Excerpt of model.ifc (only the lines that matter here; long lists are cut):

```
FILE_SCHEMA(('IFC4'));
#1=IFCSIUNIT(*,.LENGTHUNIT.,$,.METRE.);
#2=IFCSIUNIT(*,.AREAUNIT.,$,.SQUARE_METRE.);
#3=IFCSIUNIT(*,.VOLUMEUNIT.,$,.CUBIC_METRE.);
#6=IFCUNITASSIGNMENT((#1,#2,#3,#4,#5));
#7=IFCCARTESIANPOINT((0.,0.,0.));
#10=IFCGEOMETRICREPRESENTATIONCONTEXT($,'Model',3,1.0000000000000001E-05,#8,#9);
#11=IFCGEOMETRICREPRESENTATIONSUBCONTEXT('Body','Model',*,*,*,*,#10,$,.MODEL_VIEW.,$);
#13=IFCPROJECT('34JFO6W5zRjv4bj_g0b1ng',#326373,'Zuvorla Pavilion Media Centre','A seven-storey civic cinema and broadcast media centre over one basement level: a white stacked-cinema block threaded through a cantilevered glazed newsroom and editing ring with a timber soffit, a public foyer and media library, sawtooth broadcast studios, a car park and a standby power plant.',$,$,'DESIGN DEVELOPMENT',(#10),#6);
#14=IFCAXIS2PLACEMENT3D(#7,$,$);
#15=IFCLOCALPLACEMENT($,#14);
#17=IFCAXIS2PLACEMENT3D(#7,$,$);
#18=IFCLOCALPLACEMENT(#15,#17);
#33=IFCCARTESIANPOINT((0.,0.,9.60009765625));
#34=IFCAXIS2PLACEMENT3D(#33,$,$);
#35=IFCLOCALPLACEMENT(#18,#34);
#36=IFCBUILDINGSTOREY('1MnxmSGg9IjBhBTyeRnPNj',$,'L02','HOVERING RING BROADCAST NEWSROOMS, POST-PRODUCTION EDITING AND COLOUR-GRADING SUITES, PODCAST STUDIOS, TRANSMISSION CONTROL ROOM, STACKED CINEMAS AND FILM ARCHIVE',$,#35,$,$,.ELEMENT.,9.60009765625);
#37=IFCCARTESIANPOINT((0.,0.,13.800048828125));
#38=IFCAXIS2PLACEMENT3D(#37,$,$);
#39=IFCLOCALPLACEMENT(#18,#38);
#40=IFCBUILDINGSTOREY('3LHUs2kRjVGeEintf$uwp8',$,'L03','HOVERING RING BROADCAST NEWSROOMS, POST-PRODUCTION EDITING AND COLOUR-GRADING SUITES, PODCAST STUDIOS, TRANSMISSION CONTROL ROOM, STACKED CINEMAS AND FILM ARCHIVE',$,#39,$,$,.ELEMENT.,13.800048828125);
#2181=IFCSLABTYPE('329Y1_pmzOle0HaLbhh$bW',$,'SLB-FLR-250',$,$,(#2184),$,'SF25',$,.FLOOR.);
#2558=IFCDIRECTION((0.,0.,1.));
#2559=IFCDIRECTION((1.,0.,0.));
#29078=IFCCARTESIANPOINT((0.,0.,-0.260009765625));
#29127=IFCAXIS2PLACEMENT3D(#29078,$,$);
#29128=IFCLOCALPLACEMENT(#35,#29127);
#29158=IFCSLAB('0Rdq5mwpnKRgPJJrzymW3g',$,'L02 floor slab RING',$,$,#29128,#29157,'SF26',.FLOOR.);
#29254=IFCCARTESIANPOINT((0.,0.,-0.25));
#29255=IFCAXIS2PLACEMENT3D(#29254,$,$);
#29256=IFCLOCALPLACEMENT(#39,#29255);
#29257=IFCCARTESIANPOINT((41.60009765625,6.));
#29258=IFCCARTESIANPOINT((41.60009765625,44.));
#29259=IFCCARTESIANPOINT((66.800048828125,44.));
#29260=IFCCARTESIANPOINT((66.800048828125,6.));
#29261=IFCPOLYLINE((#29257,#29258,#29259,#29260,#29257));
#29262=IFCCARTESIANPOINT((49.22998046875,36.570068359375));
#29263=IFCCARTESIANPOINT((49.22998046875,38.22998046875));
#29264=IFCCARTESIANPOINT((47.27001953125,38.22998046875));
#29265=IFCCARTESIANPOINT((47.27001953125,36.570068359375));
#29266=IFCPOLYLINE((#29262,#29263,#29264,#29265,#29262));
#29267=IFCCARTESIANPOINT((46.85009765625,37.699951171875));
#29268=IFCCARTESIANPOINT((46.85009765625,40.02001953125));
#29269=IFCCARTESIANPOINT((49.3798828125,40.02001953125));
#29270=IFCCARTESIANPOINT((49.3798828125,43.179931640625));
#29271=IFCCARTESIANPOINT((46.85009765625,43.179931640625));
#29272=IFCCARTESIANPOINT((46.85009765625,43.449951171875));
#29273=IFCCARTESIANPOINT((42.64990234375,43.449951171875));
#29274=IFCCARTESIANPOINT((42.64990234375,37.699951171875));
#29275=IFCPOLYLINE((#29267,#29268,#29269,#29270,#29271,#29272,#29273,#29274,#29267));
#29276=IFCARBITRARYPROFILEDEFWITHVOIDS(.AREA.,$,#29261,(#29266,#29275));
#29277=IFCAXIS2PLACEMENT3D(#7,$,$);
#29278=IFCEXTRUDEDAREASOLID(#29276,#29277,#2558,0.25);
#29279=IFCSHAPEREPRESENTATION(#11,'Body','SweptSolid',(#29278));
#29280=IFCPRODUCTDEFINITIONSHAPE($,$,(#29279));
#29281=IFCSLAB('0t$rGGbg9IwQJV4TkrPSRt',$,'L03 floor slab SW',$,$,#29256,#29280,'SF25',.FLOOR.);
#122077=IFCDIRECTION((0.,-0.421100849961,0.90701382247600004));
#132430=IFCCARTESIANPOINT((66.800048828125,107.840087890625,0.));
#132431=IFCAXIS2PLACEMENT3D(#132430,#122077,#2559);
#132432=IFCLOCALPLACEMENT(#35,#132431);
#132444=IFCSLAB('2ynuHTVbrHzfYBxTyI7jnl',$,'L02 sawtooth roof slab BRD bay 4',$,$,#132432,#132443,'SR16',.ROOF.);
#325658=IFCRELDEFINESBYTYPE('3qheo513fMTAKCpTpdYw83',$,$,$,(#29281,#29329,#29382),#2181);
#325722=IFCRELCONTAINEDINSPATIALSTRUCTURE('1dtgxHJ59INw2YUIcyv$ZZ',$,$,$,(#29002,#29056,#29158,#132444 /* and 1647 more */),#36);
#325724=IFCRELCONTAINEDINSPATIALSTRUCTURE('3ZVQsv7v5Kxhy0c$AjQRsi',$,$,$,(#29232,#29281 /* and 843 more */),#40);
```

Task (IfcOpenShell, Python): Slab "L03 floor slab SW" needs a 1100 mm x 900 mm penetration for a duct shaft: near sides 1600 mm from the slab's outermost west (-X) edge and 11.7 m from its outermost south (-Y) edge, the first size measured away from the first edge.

```python
import numpy as np
import ifcopenshell
import ifcopenshell.api.feature
import ifcopenshell.api.geometry
import ifcopenshell.api.root
import ifcopenshell.geom
import ifcopenshell.util.placement
import ifcopenshell.util.representation
import ifcopenshell.util.shape
import ifcopenshell.util.unit

model = ifcopenshell.open("model.ifc")
unit_scale = ifcopenshell.util.unit.calculate_unit_scale(model)
settings = ifcopenshell.geom.settings()


def volume(element):
    """Net volume in cubic metres, openings subtracted."""
    shape = ifcopenshell.geom.create_shape(settings, element)
    return ifcopenshell.util.shape.get_volume(shape.geometry)


slab = model.by_guid("0t$rGGbg9IwQJV4TkrPSRt")
before = volume(slab)

# Extent in the slab's own axes, in metres. The edges named are its -X and -Y sides.
slab_shape = ifcopenshell.geom.create_shape(settings, slab)
vertices = ifcopenshell.util.shape.get_vertices(slab_shape.geometry)
x_min, y_min, bottom = vertices.min(axis=0)
top = vertices[:, 2].max()

opening = ifcopenshell.api.root.create_entity(model, ifc_class="IfcOpeningElement", name="Duct shaft opening", predefined_type="OPENING")
context = ifcopenshell.util.representation.get_context(model, "Model", "Body", "MODEL_VIEW")
width, depth = 1.1, 0.9
outline = [(0.0, 0.0), (width, 0.0), (width, depth), (0.0, depth), (0.0, 0.0)]
# Overshoot both faces by 50 mm so the cut is clean.
shape = ifcopenshell.api.geometry.add_slab_representation(
    model, context=context, depth=top - bottom + 0.1, polyline=outline
)
ifcopenshell.api.geometry.assign_representation(model, product=opening, representation=shape)

matrix = ifcopenshell.util.placement.get_local_placement(slab.ObjectPlacement)
matrix[:, 3] = matrix @ np.append(np.array([x_min + 1.6, y_min + 11.7, bottom - 0.05]) / unit_scale, 1.0)
ifcopenshell.api.geometry.edit_object_placement(model, product=opening, matrix=matrix, is_si=False)
ifcopenshell.api.feature.add_feature(model, feature=opening, element=slab)

after = volume(slab)

print(f"slab volume {before:.3f} -> {after:.3f} m3")

model.write("model_rev.ifc")
```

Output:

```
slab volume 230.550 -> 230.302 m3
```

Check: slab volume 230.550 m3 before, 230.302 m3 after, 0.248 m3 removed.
